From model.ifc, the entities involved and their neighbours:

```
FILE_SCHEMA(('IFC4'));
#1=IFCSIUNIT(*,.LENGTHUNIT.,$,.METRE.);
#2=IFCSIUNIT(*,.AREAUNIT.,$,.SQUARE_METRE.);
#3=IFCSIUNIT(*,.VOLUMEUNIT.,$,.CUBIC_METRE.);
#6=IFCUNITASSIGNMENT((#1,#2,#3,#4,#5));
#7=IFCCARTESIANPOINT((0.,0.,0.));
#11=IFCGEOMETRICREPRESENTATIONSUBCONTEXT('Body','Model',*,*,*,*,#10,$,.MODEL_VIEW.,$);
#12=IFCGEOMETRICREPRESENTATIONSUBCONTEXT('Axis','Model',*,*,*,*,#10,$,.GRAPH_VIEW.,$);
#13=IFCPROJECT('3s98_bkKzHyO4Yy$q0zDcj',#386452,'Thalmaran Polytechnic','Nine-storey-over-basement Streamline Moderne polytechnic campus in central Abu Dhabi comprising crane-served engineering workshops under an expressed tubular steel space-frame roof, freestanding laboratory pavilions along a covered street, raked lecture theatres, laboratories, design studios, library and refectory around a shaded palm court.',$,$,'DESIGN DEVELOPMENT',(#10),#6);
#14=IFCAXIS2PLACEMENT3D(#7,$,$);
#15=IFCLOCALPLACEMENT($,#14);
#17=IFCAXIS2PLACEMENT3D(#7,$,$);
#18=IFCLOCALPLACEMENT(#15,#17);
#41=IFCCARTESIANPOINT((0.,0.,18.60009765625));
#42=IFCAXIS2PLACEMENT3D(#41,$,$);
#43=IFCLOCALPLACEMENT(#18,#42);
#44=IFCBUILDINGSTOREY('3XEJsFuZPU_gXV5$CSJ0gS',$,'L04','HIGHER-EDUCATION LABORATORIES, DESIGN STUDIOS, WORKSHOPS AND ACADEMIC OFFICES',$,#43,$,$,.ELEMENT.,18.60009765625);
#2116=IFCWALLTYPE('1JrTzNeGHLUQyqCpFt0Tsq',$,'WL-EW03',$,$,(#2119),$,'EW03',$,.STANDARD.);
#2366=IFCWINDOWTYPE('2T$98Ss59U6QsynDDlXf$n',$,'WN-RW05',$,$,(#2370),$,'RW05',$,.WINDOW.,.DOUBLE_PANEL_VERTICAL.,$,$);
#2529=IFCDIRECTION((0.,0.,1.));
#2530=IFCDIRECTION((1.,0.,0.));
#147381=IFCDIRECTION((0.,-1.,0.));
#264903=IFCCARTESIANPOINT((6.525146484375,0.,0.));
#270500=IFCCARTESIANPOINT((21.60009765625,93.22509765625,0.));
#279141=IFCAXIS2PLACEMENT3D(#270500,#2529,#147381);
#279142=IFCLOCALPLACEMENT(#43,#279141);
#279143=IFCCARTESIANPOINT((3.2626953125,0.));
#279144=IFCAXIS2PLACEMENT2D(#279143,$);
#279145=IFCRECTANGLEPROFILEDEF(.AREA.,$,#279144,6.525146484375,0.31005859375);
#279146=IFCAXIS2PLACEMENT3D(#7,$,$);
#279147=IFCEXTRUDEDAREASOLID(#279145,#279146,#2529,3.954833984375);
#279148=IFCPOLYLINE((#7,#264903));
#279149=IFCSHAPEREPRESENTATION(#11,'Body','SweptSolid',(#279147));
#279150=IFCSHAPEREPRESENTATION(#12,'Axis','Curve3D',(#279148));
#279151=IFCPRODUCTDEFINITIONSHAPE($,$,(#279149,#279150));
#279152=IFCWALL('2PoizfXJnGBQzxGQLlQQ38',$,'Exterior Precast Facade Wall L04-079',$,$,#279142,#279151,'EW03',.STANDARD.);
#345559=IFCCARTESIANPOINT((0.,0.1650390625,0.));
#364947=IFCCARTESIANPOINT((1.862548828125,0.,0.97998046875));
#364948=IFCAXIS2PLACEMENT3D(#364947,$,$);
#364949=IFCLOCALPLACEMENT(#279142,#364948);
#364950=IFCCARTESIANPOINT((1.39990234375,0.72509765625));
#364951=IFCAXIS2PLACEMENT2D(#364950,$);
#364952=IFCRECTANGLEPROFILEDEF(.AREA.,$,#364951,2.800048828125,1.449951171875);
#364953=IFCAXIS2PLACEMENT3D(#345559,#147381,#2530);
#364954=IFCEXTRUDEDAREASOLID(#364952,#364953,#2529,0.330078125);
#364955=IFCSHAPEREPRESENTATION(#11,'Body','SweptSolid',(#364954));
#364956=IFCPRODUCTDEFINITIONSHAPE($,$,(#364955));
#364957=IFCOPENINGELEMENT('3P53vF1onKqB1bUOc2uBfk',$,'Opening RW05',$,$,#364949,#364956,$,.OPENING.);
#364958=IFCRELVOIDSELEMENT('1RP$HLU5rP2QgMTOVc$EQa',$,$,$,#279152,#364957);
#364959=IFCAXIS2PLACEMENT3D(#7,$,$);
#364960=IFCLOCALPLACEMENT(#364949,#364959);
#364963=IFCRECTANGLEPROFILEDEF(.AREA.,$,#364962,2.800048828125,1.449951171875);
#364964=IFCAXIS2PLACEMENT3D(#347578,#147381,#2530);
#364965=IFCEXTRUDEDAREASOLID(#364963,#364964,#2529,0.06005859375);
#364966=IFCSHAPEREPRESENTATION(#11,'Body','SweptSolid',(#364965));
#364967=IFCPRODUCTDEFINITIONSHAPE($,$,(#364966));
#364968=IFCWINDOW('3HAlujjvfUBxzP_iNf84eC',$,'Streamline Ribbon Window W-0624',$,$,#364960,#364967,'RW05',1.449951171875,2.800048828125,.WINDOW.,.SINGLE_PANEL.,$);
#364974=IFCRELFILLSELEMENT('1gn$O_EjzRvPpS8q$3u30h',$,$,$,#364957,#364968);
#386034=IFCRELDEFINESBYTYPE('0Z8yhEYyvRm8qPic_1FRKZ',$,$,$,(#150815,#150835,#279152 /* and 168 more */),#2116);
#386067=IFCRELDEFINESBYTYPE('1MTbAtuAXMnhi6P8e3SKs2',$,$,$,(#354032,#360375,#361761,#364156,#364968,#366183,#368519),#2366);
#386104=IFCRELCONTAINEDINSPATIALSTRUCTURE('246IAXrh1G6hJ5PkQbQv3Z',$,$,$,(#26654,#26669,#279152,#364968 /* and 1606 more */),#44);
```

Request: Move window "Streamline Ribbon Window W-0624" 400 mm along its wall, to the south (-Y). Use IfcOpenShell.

```python
import ifcopenshell
import ifcopenshell.api.geometry
import ifcopenshell.util.placement
import ifcopenshell.util.unit

model = ifcopenshell.open("model.ifc")
unit_scale = ifcopenshell.util.unit.calculate_unit_scale(model)

window = model.by_guid("3HAlujjvfUBxzP_iNf84eC")
opening = window.FillsVoids[0].RelatingOpeningElement
wall = opening.VoidsElements[0].RelatingBuildingElement

wall_matrix = ifcopenshell.util.placement.get_local_placement(wall.ObjectPlacement)
shift = wall_matrix[:3, 0] * 0.4 / unit_scale
before = ifcopenshell.util.placement.get_local_placement(window.ObjectPlacement)[:3, 3].copy()

# The window is placed relative to its opening, so it follows when the opening moves.
matrix = ifcopenshell.util.placement.get_local_placement(opening.ObjectPlacement)
matrix[:3, 3] += shift
ifcopenshell.api.geometry.edit_object_placement(
    model, product=opening, matrix=matrix, is_si=False, should_transform_children=True
)

after = ifcopenshell.util.placement.get_local_placement(window.ObjectPlacement)[:3, 3]
print("window moved by", (after - before).round(3) + 0.0)

model.write("model_edited.ifc")
```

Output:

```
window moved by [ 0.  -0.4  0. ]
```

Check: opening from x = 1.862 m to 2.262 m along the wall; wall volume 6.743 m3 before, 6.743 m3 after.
